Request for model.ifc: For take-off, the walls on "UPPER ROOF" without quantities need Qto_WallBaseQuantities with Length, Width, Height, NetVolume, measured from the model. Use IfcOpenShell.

First a look at what the model holds.

```python
import ifcopenshell
import ifcopenshell.util.element
import ifcopenshell.util.unit

model = ifcopenshell.open("model.ifc")
print(model.schema)
for unit_type in ("LENGTHUNIT", "AREAUNIT", "VOLUMEUNIT"):
    print(unit_type, ifcopenshell.util.unit.calculate_unit_scale(model, unit_type))
storey = next(s for s in model.by_type("IfcBuildingStorey") if s.Name == "UPPER ROOF")
walls = [e for e in ifcopenshell.util.element.get_decomposition(storey) if e.is_a("IfcWall")]
for e in sorted(walls, key=lambda e: e.id()):
    print(e.id(), e.is_a(), e.Name, list(ifcopenshell.util.element.get_psets(e, qtos_only=True)), sep=" | ")
```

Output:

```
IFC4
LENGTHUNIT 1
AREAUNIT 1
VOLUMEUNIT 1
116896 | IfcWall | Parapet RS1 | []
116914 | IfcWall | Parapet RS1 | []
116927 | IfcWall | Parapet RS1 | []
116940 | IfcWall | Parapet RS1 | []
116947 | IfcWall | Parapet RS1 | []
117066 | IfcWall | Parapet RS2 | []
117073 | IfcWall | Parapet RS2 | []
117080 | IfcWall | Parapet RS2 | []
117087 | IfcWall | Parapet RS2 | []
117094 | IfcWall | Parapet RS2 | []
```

```python
import ifcopenshell
import ifcopenshell.api.pset
import ifcopenshell.geom
import ifcopenshell.util.element
import ifcopenshell.util.shape
import ifcopenshell.util.unit

model = ifcopenshell.open("model.ifc")
unit_scale = ifcopenshell.util.unit.calculate_unit_scale(model)
volume_scale = ifcopenshell.util.unit.calculate_unit_scale(model, "VOLUMEUNIT")
settings = ifcopenshell.geom.settings()

storey = next(s for s in model.by_type("IfcBuildingStorey") if s.Name == "UPPER ROOF")
walls = [e for e in ifcopenshell.util.element.get_decomposition(storey) if e.is_a("IfcWall")]

for e in sorted(walls, key=lambda e: e.id()):
    if ifcopenshell.util.element.get_psets(e, qtos_only=True, should_inherit=False):
        continue
    # Geometry comes back in metres, in the element's own axes.
    shape = ifcopenshell.geom.create_shape(settings, e)
    values = {
        "Length": ifcopenshell.util.shape.get_x(shape.geometry) / unit_scale,
        "Width": ifcopenshell.util.shape.get_y(shape.geometry) / unit_scale,
        "Height": ifcopenshell.util.shape.get_z(shape.geometry) / unit_scale,
        "NetVolume": ifcopenshell.util.shape.get_volume(shape.geometry) / volume_scale,
    }
    qto = ifcopenshell.api.pset.add_qto(model, product=e, name="Qto_WallBaseQuantities")
    ifcopenshell.api.pset.edit_qto(model, qto=qto, properties=values)
    print(e.id(), {k: round(v, 3) for k, v in values.items()})

model.write("model_v2.ifc")
```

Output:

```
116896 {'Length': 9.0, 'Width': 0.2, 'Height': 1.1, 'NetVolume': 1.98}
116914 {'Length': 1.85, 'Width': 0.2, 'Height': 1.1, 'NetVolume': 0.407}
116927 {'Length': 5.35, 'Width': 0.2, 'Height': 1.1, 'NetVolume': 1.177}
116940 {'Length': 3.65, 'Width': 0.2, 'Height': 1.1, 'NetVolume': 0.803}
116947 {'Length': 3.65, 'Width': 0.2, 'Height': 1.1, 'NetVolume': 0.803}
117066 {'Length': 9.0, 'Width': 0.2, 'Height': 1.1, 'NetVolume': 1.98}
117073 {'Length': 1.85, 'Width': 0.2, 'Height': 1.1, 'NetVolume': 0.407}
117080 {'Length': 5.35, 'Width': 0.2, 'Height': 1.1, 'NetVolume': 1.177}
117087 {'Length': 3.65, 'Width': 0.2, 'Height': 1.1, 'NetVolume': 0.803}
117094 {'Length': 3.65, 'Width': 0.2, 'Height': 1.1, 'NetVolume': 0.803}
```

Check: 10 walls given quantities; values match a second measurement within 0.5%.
